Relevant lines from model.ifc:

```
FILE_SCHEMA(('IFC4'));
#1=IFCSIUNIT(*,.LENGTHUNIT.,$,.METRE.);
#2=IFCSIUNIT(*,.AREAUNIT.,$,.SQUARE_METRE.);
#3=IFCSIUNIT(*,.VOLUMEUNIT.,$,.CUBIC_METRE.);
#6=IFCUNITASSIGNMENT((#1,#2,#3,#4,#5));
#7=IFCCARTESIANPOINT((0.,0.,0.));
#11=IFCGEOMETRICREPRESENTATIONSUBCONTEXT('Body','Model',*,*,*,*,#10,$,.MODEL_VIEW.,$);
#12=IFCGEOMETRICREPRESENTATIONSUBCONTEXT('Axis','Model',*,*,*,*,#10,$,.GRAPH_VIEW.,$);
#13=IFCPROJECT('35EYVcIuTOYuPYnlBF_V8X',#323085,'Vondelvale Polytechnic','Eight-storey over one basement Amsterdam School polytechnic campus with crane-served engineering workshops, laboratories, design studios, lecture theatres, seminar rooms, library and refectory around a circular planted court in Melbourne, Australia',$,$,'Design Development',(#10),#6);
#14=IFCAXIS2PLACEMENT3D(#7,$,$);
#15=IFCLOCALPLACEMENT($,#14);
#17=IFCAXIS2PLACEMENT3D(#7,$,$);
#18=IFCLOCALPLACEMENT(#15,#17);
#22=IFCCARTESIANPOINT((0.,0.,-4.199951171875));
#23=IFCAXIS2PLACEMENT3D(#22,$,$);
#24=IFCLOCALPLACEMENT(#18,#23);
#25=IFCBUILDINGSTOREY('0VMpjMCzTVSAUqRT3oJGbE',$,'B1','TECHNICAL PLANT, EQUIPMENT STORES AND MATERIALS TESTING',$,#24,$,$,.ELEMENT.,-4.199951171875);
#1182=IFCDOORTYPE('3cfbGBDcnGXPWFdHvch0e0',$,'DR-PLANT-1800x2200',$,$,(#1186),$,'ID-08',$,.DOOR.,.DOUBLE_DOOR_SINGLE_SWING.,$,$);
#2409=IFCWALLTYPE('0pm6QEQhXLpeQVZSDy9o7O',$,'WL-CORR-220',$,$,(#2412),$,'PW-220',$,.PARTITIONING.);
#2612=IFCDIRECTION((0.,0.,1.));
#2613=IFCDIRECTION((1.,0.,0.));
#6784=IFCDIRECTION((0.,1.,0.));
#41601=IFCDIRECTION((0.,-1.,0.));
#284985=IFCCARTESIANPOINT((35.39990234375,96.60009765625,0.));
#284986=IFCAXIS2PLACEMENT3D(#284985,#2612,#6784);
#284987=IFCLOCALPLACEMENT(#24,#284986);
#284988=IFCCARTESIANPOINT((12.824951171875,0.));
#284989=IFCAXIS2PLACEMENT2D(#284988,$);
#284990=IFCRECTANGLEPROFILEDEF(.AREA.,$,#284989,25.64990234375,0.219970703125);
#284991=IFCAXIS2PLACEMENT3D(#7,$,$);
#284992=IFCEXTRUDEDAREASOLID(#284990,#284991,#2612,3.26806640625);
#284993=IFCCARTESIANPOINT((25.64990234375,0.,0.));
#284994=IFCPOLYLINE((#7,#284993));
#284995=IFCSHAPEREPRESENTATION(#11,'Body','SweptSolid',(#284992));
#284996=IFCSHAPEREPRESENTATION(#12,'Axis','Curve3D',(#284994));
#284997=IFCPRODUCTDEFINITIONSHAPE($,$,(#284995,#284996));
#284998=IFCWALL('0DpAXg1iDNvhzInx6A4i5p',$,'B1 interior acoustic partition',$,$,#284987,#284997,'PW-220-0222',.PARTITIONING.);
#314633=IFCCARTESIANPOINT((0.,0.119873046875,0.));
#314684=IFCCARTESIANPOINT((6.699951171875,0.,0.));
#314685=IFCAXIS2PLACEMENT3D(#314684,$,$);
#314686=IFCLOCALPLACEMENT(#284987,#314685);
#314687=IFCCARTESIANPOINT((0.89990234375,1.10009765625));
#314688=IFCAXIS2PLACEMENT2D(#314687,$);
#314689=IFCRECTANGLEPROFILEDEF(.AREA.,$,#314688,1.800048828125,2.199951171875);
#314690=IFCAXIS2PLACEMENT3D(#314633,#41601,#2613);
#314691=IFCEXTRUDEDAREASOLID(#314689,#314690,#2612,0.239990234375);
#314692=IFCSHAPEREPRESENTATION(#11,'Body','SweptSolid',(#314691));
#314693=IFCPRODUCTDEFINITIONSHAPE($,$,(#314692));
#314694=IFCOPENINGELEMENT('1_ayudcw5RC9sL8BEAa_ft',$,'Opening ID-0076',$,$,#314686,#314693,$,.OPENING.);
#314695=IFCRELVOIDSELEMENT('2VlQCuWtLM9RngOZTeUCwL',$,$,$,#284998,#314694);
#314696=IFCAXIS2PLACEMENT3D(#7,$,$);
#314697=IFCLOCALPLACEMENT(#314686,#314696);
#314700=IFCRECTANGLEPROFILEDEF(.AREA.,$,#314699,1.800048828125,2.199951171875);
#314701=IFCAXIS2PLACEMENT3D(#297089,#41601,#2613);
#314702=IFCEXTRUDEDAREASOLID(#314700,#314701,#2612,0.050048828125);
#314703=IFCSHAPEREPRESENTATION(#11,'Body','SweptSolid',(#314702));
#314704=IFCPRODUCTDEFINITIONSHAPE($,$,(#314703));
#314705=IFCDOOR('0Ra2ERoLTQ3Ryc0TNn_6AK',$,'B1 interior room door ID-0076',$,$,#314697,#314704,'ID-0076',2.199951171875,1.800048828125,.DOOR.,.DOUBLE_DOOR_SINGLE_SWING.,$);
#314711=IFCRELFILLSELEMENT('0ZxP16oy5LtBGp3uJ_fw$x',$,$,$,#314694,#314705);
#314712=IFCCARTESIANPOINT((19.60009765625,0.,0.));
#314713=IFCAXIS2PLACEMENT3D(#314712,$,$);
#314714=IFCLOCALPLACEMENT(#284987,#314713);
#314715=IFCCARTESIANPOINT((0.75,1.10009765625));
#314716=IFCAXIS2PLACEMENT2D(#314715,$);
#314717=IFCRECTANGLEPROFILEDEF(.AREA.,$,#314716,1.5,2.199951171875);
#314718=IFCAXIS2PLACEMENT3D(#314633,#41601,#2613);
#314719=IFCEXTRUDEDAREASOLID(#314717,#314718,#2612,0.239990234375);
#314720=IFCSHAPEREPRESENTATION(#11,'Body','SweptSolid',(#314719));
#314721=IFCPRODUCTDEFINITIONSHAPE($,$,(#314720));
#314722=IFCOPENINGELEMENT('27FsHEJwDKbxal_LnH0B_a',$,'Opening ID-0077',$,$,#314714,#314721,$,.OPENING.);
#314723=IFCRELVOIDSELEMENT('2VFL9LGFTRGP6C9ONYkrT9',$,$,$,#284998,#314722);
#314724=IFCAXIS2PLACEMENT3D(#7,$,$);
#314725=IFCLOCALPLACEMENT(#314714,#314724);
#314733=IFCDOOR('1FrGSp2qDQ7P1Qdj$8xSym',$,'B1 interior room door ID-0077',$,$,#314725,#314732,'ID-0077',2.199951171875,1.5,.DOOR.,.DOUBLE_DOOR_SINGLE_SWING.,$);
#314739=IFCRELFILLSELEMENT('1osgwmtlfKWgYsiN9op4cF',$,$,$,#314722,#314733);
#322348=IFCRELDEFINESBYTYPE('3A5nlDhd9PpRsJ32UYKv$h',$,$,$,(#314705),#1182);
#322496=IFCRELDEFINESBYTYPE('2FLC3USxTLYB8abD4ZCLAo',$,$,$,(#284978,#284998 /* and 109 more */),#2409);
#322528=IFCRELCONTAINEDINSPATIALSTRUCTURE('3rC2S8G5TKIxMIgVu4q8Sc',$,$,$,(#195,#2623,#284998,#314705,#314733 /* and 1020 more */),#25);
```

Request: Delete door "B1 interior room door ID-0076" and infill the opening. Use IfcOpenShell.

```python
import ifcopenshell
import ifcopenshell.api.feature
import ifcopenshell.api.root
import ifcopenshell.geom
import ifcopenshell.util.shape

model = ifcopenshell.open("model.ifc")
settings = ifcopenshell.geom.settings()


def volume(element):
    """Net volume in cubic metres, openings subtracted."""
    shape = ifcopenshell.geom.create_shape(settings, element)
    return ifcopenshell.util.shape.get_volume(shape.geometry)


door = model.by_guid("0Ra2ERoLTQ3Ryc0TNn_6AK")
opening = door.FillsVoids[0].RelatingOpeningElement
wall = opening.VoidsElements[0].RelatingBuildingElement
before = volume(wall)

ifcopenshell.api.root.remove_product(model, product=door)
ifcopenshell.api.feature.remove_feature(model, feature=opening)

after = volume(wall)

print(f"wall volume {before:.3f} -> {after:.3f} m3")

model.write("model-out.ifc")
```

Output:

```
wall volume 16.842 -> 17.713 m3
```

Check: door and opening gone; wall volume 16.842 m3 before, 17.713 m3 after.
